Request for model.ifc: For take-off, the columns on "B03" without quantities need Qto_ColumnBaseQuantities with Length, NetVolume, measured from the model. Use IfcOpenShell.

First a look at what the model holds.

```python
import ifcopenshell
import ifcopenshell.util.element
import ifcopenshell.util.unit

model = ifcopenshell.open("model.ifc")
print(model.schema)
for unit_type in ("LENGTHUNIT", "AREAUNIT", "VOLUMEUNIT"):
    print(unit_type, ifcopenshell.util.unit.calculate_unit_scale(model, unit_type))
storey = next(s for s in model.by_type("IfcBuildingStorey") if s.Name == "B03")
columns = [e for e in ifcopenshell.util.element.get_decomposition(storey) if e.is_a("IfcColumn")]
for e in sorted(columns, key=lambda e: e.id()):
    print(e.id(), e.is_a(), e.Name, list(ifcopenshell.util.element.get_psets(e, qtos_only=True)), sep=" | ")
```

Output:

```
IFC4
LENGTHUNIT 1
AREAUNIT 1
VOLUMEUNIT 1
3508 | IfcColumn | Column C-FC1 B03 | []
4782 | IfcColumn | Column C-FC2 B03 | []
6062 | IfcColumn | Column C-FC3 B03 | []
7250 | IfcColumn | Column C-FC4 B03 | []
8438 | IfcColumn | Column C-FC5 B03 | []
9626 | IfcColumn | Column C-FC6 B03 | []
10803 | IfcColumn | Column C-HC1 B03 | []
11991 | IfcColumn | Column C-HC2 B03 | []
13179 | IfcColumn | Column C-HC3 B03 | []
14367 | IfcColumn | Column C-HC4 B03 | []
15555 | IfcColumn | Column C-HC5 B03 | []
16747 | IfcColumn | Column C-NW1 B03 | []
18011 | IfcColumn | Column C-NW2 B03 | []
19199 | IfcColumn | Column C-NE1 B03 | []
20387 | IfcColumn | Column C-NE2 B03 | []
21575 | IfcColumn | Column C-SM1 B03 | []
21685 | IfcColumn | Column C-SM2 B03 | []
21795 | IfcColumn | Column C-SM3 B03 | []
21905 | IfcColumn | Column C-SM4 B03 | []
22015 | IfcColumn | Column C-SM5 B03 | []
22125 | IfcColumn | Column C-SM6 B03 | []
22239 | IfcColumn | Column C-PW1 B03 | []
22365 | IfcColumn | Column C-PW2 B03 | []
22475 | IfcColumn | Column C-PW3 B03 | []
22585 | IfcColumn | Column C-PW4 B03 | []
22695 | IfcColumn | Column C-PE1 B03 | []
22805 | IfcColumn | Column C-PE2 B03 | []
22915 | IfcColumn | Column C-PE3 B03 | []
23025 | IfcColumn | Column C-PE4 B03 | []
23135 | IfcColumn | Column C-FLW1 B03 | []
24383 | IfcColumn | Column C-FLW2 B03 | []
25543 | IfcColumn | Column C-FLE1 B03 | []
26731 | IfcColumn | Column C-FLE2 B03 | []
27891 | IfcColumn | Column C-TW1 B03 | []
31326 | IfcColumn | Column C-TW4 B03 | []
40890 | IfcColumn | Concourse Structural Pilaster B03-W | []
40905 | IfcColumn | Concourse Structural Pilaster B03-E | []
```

```python
import ifcopenshell
import ifcopenshell.api.pset
import ifcopenshell.geom
import ifcopenshell.util.element
import ifcopenshell.util.shape
import ifcopenshell.util.unit

model = ifcopenshell.open("model.ifc")
unit_scale = ifcopenshell.util.unit.calculate_unit_scale(model)
volume_scale = ifcopenshell.util.unit.calculate_unit_scale(model, "VOLUMEUNIT")
settings = ifcopenshell.geom.settings()

storey = next(s for s in model.by_type("IfcBuildingStorey") if s.Name == "B03")
columns = [e for e in ifcopenshell.util.element.get_decomposition(storey) if e.is_a("IfcColumn")]

for e in sorted(columns, key=lambda e: e.id()):
    if ifcopenshell.util.element.get_psets(e, qtos_only=True, should_inherit=False):
        continue
    # Geometry comes back in metres, in the element's own axes.
    shape = ifcopenshell.geom.create_shape(settings, e)
    values = {
        "Length": ifcopenshell.util.shape.get_z(shape.geometry) / unit_scale,
        "NetVolume": ifcopenshell.util.shape.get_volume(shape.geometry) / volume_scale,
    }
    qto = ifcopenshell.api.pset.add_qto(model, product=e, name="Qto_ColumnBaseQuantities")
    ifcopenshell.api.pset.edit_qto(model, qto=qto, properties=values)
    print(e.id(), {k: round(v, 3) for k, v in values.items()})

model.write("model_edited.ifc")
```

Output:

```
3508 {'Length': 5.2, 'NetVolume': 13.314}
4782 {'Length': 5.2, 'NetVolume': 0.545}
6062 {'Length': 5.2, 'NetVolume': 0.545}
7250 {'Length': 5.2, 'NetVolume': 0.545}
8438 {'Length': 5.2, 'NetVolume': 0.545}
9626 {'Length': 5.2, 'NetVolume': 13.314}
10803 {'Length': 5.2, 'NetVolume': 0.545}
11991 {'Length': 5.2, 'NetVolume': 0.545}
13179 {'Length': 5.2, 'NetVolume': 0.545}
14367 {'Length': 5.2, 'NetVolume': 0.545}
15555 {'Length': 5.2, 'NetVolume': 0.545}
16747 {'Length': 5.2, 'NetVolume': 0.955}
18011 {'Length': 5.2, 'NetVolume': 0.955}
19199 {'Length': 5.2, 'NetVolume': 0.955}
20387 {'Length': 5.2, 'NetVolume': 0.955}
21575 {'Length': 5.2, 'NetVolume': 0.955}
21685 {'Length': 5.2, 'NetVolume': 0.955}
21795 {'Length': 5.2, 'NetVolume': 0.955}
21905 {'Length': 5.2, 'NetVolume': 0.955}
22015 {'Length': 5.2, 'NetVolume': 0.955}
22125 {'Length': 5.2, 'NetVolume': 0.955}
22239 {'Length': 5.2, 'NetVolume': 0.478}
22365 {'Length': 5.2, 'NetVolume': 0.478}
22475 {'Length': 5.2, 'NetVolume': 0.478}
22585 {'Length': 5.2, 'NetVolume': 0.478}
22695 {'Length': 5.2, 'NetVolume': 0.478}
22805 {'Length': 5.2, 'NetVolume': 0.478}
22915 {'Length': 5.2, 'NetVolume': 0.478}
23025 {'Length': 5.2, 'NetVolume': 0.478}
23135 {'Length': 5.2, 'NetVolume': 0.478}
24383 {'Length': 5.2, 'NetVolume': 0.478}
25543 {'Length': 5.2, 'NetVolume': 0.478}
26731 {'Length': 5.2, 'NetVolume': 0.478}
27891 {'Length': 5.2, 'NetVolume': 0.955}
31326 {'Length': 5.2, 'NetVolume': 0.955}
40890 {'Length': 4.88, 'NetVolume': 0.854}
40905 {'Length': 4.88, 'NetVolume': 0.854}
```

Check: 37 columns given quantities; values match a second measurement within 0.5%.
